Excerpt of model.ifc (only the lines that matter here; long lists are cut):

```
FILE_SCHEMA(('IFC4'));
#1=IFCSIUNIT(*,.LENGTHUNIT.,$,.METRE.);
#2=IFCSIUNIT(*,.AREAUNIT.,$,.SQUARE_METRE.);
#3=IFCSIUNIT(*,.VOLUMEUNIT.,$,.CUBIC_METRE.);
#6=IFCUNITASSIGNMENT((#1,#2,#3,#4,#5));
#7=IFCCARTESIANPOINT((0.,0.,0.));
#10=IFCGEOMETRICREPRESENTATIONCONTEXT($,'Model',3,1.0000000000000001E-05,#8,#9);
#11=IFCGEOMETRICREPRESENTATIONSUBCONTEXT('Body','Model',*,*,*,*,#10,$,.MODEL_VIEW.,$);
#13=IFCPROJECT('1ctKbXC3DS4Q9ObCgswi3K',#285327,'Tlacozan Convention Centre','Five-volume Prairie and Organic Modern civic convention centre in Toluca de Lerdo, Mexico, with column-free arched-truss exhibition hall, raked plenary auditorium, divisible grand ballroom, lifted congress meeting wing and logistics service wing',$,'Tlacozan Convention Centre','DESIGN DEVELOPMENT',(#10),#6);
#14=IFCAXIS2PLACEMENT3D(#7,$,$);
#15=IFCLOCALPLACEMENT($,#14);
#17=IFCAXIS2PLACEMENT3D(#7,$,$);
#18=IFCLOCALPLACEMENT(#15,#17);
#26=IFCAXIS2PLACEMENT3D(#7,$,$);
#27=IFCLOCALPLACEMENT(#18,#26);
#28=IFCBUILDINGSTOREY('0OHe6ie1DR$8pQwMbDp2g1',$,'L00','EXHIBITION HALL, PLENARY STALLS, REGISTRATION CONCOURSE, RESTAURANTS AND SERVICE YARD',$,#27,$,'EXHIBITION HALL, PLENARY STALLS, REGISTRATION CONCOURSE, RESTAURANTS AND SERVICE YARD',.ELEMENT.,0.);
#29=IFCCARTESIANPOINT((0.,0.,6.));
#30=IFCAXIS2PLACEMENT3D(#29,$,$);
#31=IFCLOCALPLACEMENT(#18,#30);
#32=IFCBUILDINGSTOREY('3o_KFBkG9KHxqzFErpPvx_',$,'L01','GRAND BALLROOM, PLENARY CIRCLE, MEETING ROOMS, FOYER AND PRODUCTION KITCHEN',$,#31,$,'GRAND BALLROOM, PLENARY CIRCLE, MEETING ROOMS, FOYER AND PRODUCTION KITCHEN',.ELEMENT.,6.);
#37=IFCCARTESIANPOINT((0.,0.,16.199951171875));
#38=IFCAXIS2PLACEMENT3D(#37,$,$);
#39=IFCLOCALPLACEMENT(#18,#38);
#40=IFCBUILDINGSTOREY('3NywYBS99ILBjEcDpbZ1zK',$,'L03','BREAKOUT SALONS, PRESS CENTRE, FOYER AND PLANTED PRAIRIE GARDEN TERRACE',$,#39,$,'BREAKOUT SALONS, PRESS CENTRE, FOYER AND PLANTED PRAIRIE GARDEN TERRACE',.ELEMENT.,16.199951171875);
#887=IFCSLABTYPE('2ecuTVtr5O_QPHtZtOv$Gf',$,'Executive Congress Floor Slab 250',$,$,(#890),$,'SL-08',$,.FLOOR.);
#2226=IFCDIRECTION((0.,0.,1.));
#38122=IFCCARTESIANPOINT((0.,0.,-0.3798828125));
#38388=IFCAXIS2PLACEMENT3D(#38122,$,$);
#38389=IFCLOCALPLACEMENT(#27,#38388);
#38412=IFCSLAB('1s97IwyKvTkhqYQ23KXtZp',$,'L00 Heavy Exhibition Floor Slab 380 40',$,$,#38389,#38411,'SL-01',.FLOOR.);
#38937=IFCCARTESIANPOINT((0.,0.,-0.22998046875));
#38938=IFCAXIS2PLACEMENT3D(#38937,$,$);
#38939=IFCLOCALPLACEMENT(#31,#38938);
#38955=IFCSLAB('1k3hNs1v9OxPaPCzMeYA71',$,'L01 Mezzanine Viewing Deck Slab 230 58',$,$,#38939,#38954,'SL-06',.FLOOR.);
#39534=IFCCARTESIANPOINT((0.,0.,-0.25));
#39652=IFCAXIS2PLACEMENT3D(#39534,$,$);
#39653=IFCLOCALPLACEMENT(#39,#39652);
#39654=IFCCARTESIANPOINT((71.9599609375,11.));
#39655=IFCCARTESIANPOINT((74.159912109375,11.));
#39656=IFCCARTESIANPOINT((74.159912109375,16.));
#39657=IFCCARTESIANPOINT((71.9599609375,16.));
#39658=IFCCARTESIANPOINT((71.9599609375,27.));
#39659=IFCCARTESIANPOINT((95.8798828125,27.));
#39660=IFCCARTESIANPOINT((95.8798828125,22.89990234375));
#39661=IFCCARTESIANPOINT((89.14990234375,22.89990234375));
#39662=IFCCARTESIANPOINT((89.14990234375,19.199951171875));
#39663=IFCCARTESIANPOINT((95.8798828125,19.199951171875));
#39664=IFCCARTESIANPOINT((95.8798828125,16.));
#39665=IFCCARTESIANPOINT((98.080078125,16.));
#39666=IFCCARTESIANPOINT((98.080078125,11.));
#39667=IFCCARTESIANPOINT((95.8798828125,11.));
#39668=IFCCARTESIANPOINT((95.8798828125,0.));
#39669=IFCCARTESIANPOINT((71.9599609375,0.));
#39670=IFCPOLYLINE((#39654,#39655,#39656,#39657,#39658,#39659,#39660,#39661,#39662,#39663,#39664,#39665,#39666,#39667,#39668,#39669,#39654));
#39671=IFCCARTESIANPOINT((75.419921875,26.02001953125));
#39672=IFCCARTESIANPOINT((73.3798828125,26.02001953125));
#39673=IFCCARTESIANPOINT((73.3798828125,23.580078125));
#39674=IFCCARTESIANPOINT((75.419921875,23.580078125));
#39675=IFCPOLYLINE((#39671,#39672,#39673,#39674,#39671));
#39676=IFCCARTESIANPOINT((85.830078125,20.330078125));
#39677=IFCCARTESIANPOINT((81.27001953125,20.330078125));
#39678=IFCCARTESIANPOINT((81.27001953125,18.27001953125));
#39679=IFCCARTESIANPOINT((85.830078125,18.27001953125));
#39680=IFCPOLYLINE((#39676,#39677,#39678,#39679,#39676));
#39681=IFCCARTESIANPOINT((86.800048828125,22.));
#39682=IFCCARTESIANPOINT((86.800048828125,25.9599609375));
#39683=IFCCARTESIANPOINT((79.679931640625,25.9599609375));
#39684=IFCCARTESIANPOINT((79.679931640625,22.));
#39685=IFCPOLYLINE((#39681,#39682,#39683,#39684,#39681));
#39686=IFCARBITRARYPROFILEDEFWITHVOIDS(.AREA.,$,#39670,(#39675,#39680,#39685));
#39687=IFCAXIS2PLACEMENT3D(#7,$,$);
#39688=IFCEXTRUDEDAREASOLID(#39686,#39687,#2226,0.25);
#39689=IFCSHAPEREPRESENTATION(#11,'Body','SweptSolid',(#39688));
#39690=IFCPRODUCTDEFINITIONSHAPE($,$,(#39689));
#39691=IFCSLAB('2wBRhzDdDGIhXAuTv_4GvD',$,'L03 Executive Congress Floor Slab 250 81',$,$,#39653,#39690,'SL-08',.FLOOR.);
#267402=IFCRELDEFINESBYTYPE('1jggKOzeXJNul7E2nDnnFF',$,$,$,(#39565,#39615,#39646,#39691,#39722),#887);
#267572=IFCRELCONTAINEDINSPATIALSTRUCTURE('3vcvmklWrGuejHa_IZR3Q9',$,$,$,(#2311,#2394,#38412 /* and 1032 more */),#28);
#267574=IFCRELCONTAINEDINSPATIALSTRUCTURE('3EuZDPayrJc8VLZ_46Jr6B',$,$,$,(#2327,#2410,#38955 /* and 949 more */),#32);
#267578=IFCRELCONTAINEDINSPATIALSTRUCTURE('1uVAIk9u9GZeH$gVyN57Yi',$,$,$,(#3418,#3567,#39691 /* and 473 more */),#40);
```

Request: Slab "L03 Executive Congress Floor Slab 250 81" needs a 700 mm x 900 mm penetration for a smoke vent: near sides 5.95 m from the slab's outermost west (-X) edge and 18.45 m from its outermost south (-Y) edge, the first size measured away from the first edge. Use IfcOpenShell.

```python
import numpy as np
import ifcopenshell
import ifcopenshell.api.feature
import ifcopenshell.api.geometry
import ifcopenshell.api.root
import ifcopenshell.geom
import ifcopenshell.util.placement
import ifcopenshell.util.representation
import ifcopenshell.util.shape
import ifcopenshell.util.unit

model = ifcopenshell.open("model.ifc")
unit_scale = ifcopenshell.util.unit.calculate_unit_scale(model)
settings = ifcopenshell.geom.settings()


def volume(element):
    """Net volume in cubic metres, openings subtracted."""
    shape = ifcopenshell.geom.create_shape(settings, element)
    return ifcopenshell.util.shape.get_volume(shape.geometry)


slab = model.by_id(39691)
before = volume(slab)

# Extent in the slab's own axes, in metres. The edges named are its -X and -Y sides.
slab_shape = ifcopenshell.geom.create_shape(settings, slab)
vertices = ifcopenshell.util.shape.get_vertices(slab_shape.geometry)
x_min, y_min, bottom = vertices.min(axis=0)
top = vertices[:, 2].max()

opening = ifcopenshell.api.root.create_entity(model, ifc_class="IfcOpeningElement", name="Smoke vent opening", predefined_type="OPENING")
context = ifcopenshell.util.representation.get_context(model, "Model", "Body", "MODEL_VIEW")
width, depth = 0.7, 0.9
outline = [(0.0, 0.0), (width, 0.0), (width, depth), (0.0, depth), (0.0, 0.0)]
# Overshoot both faces by 50 mm so the cut is clean.
shape = ifcopenshell.api.geometry.add_slab_representation(
    model, context=context, depth=top - bottom + 0.1, polyline=outline
)
ifcopenshell.api.geometry.assign_representation(model, product=opening, representation=shape)

matrix = ifcopenshell.util.placement.get_local_placement(slab.ObjectPlacement)
matrix[:, 3] = matrix @ np.append(np.array([x_min + 5.95, y_min + 18.45, bottom - 0.05]) / unit_scale, 1.0)
ifcopenshell.api.geometry.edit_object_placement(model, product=opening, matrix=matrix, is_si=False)
ifcopenshell.api.feature.add_feature(model, feature=opening, element=slab)

after = volume(slab)

print(f"slab volume {before:.3f} -> {after:.3f} m3")

model.write("model_v2.ifc")
```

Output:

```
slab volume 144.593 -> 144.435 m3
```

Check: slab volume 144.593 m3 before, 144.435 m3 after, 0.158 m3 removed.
